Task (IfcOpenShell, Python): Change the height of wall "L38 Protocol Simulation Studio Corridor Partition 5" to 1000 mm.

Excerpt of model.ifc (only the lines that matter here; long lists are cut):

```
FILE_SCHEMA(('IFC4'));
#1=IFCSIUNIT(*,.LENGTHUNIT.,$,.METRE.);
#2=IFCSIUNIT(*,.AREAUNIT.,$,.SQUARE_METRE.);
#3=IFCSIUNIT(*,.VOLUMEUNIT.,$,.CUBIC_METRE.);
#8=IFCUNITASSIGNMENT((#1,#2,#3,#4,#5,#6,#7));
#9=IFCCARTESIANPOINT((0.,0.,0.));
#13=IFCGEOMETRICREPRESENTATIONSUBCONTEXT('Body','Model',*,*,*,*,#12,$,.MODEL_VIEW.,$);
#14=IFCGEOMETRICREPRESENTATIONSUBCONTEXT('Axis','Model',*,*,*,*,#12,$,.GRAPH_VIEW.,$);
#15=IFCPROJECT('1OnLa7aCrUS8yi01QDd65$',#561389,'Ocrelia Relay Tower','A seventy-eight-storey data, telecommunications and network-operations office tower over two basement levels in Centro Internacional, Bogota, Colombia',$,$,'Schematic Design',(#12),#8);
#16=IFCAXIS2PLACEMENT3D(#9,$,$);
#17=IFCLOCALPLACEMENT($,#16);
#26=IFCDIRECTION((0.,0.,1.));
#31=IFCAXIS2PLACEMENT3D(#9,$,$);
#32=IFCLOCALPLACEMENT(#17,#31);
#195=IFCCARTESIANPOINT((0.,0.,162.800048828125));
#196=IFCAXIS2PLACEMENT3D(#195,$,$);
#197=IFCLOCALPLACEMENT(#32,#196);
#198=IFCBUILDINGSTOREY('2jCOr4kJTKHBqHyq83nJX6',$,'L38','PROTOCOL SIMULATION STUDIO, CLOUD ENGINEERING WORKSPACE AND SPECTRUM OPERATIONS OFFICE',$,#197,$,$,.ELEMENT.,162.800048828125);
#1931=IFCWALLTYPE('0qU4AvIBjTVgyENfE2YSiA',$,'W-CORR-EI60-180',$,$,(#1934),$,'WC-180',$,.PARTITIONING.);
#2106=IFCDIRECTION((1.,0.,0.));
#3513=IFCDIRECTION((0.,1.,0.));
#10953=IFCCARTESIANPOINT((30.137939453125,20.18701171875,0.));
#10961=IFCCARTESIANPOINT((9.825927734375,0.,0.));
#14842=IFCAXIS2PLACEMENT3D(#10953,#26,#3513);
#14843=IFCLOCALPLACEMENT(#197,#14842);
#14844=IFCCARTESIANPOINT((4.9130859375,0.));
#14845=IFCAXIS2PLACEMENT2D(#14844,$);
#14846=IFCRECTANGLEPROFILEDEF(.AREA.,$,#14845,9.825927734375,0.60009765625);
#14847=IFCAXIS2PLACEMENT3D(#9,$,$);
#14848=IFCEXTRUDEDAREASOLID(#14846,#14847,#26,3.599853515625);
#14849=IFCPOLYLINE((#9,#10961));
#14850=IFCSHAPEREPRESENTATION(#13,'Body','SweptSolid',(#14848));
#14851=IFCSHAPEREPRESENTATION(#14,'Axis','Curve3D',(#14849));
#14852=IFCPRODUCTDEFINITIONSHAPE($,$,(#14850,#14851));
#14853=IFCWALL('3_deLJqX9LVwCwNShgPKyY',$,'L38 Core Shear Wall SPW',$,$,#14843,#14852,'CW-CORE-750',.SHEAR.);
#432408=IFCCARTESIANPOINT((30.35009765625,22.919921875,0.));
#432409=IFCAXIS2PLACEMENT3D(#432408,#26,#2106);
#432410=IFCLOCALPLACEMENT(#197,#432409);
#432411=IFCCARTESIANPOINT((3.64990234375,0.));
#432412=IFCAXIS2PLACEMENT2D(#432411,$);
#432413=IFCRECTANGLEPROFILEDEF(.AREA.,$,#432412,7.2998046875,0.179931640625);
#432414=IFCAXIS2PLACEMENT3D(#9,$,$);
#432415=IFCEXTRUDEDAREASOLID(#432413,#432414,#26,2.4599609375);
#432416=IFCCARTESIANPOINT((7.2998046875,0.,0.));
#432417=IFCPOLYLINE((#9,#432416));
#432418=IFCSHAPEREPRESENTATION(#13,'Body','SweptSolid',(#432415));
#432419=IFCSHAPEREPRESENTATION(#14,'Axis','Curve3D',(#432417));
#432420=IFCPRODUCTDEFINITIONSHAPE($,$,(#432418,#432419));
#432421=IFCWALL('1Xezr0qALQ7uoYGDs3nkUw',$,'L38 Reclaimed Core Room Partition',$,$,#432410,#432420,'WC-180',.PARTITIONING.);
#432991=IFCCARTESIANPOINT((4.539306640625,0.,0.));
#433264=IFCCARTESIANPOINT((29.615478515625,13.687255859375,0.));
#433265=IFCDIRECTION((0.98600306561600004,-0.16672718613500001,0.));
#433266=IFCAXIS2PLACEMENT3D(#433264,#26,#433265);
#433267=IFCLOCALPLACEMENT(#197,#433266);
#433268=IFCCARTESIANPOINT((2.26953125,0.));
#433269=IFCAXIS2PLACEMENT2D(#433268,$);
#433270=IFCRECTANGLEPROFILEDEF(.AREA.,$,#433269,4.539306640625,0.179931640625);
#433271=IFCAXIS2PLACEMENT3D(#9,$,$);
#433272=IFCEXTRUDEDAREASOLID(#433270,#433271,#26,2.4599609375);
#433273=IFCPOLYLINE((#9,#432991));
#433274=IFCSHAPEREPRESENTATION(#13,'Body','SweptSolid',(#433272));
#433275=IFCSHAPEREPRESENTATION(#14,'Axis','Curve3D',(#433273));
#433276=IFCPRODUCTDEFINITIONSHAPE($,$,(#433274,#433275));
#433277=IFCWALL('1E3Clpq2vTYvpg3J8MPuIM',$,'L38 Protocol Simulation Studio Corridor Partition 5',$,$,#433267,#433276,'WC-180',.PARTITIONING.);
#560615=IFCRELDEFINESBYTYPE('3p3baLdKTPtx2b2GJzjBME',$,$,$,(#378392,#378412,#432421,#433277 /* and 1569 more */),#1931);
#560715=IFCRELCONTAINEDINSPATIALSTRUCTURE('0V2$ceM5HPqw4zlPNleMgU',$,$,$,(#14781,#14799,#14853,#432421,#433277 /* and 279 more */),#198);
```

```python
import ifcopenshell
import ifcopenshell.geom
import ifcopenshell.util.representation
import ifcopenshell.util.shape
import ifcopenshell.util.unit

model = ifcopenshell.open("model.ifc")
unit_scale = ifcopenshell.util.unit.calculate_unit_scale(model)
settings = ifcopenshell.geom.settings()


def volume(element):
    """Net volume in cubic metres, openings subtracted."""
    shape = ifcopenshell.geom.create_shape(settings, element)
    return ifcopenshell.util.shape.get_volume(shape.geometry)


wall = model.by_guid("1E3Clpq2vTYvpg3J8MPuIM")
before = volume(wall)

body = ifcopenshell.util.representation.get_representation(wall, "Model", "Body")
solid = body.Items[0]
old_height = solid.Depth
solid.Depth = 1 / unit_scale
after = volume(wall)

print(f"height {old_height:g} -> {solid.Depth:g}, volume {before:.3f} -> {after:.3f} m3")

model.write("model_updated.ifc")
```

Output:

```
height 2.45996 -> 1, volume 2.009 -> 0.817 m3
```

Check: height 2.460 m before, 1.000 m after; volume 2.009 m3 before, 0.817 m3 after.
